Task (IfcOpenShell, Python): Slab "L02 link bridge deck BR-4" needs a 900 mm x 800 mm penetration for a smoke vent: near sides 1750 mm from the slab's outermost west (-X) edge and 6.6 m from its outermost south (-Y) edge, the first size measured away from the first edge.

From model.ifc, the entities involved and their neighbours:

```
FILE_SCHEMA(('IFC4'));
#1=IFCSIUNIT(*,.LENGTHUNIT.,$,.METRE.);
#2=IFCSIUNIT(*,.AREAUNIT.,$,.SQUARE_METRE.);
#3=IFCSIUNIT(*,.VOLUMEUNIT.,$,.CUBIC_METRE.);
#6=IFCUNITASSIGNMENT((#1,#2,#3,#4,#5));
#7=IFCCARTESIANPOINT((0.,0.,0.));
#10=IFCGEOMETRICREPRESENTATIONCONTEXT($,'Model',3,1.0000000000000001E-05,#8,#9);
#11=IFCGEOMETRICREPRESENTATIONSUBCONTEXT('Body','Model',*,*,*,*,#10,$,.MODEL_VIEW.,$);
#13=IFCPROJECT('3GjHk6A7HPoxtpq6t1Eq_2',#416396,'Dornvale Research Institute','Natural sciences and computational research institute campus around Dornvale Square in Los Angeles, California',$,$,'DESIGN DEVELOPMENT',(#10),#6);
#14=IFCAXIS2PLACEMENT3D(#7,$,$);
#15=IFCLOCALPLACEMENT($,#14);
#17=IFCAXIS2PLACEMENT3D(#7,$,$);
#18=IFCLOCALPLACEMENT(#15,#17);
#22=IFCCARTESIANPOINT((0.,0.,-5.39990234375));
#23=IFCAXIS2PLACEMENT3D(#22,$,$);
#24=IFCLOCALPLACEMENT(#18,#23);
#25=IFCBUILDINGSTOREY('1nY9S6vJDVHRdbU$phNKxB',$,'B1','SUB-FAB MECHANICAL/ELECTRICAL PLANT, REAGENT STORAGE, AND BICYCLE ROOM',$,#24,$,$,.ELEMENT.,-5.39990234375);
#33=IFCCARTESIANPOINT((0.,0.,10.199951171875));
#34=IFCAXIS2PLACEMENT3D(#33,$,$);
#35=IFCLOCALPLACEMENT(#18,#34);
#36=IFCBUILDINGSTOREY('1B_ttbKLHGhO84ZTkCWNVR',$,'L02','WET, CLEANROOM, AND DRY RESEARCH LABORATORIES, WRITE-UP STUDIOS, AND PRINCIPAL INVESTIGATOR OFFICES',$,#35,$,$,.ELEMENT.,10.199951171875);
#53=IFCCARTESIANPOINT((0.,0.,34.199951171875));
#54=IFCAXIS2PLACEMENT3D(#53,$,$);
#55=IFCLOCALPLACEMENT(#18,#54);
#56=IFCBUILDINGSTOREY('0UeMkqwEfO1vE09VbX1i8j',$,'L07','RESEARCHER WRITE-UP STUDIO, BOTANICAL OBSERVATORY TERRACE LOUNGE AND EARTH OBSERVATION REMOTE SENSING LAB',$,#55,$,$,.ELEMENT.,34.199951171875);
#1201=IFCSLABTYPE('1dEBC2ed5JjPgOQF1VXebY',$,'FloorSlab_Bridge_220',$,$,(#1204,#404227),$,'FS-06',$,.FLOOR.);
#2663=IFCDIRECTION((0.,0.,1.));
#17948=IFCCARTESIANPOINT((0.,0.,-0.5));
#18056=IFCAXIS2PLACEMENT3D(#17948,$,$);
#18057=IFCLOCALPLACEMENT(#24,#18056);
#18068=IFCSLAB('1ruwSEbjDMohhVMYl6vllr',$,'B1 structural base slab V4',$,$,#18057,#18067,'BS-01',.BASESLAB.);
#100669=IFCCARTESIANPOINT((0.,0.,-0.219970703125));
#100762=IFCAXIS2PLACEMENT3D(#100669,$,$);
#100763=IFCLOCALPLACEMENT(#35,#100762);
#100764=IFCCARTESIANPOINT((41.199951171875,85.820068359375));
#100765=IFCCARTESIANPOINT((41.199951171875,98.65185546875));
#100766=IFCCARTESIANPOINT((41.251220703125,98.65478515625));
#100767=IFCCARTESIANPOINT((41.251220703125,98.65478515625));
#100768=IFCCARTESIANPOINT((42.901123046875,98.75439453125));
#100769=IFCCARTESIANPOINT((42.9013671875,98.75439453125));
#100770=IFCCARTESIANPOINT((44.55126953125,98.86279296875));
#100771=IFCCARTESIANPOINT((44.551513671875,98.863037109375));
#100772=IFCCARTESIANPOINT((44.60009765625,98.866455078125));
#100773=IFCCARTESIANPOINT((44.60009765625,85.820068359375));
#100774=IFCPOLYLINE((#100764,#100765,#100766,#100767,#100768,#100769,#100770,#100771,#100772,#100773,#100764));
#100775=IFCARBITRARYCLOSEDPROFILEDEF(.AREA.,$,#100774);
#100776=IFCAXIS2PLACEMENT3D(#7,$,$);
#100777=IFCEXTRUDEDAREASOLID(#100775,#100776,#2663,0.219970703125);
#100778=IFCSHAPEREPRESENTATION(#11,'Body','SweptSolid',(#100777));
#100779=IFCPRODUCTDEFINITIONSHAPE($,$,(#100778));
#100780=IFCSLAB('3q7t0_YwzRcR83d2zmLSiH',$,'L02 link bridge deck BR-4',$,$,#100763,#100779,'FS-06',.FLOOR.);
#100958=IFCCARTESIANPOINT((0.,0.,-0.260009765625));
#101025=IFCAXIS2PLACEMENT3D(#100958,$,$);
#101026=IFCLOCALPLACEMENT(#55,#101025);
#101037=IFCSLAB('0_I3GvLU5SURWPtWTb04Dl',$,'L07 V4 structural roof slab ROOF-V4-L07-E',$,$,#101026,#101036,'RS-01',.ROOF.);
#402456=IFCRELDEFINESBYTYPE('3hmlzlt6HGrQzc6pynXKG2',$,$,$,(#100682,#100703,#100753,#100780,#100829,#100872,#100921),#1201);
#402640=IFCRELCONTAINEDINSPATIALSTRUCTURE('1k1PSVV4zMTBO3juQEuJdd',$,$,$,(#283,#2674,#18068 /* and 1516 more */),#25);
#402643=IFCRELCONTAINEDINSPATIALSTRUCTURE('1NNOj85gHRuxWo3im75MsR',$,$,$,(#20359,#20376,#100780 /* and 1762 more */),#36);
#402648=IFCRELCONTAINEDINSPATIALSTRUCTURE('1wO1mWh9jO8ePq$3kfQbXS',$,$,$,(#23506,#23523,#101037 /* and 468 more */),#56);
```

```python
import numpy as np
import ifcopenshell
import ifcopenshell.api.feature
import ifcopenshell.api.geometry
import ifcopenshell.api.root
import ifcopenshell.geom
import ifcopenshell.util.placement
import ifcopenshell.util.representation
import ifcopenshell.util.shape
import ifcopenshell.util.unit

model = ifcopenshell.open("model.ifc")
unit_scale = ifcopenshell.util.unit.calculate_unit_scale(model)
settings = ifcopenshell.geom.settings()


def volume(element):
    """Net volume in cubic metres, openings subtracted."""
    shape = ifcopenshell.geom.create_shape(settings, element)
    return ifcopenshell.util.shape.get_volume(shape.geometry)


slab = model.by_id(100780)
before = volume(slab)

# Extent in the slab's own axes, in metres. The edges named are its -X and -Y sides.
slab_shape = ifcopenshell.geom.create_shape(settings, slab)
vertices = ifcopenshell.util.shape.get_vertices(slab_shape.geometry)
x_min, y_min, bottom = vertices.min(axis=0)
top = vertices[:, 2].max()

opening = ifcopenshell.api.root.create_entity(model, ifc_class="IfcOpeningElement", name="Smoke vent opening", predefined_type="OPENING")
context = ifcopenshell.util.representation.get_context(model, "Model", "Body", "MODEL_VIEW")
width, depth = 0.9, 0.8
outline = [(0.0, 0.0), (width, 0.0), (width, depth), (0.0, depth), (0.0, 0.0)]
# Overshoot both faces by 50 mm so the cut is clean.
shape = ifcopenshell.api.geometry.add_slab_representation(
    model, context=context, depth=top - bottom + 0.1, polyline=outline
)
ifcopenshell.api.geometry.assign_representation(model, product=opening, representation=shape)

matrix = ifcopenshell.util.placement.get_local_placement(slab.ObjectPlacement)
matrix[:, 3] = matrix @ np.append(np.array([x_min + 1.75, y_min + 6.6, bottom - 0.05]) / unit_scale, 1.0)
ifcopenshell.api.geometry.edit_object_placement(model, product=opening, matrix=matrix, is_si=False)
ifcopenshell.api.feature.add_feature(model, feature=opening, element=slab)

after = volume(slab)

print(f"slab volume {before:.3f} -> {after:.3f} m3")

model.write("model-out.ifc")
```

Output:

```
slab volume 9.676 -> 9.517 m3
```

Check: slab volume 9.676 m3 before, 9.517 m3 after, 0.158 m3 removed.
